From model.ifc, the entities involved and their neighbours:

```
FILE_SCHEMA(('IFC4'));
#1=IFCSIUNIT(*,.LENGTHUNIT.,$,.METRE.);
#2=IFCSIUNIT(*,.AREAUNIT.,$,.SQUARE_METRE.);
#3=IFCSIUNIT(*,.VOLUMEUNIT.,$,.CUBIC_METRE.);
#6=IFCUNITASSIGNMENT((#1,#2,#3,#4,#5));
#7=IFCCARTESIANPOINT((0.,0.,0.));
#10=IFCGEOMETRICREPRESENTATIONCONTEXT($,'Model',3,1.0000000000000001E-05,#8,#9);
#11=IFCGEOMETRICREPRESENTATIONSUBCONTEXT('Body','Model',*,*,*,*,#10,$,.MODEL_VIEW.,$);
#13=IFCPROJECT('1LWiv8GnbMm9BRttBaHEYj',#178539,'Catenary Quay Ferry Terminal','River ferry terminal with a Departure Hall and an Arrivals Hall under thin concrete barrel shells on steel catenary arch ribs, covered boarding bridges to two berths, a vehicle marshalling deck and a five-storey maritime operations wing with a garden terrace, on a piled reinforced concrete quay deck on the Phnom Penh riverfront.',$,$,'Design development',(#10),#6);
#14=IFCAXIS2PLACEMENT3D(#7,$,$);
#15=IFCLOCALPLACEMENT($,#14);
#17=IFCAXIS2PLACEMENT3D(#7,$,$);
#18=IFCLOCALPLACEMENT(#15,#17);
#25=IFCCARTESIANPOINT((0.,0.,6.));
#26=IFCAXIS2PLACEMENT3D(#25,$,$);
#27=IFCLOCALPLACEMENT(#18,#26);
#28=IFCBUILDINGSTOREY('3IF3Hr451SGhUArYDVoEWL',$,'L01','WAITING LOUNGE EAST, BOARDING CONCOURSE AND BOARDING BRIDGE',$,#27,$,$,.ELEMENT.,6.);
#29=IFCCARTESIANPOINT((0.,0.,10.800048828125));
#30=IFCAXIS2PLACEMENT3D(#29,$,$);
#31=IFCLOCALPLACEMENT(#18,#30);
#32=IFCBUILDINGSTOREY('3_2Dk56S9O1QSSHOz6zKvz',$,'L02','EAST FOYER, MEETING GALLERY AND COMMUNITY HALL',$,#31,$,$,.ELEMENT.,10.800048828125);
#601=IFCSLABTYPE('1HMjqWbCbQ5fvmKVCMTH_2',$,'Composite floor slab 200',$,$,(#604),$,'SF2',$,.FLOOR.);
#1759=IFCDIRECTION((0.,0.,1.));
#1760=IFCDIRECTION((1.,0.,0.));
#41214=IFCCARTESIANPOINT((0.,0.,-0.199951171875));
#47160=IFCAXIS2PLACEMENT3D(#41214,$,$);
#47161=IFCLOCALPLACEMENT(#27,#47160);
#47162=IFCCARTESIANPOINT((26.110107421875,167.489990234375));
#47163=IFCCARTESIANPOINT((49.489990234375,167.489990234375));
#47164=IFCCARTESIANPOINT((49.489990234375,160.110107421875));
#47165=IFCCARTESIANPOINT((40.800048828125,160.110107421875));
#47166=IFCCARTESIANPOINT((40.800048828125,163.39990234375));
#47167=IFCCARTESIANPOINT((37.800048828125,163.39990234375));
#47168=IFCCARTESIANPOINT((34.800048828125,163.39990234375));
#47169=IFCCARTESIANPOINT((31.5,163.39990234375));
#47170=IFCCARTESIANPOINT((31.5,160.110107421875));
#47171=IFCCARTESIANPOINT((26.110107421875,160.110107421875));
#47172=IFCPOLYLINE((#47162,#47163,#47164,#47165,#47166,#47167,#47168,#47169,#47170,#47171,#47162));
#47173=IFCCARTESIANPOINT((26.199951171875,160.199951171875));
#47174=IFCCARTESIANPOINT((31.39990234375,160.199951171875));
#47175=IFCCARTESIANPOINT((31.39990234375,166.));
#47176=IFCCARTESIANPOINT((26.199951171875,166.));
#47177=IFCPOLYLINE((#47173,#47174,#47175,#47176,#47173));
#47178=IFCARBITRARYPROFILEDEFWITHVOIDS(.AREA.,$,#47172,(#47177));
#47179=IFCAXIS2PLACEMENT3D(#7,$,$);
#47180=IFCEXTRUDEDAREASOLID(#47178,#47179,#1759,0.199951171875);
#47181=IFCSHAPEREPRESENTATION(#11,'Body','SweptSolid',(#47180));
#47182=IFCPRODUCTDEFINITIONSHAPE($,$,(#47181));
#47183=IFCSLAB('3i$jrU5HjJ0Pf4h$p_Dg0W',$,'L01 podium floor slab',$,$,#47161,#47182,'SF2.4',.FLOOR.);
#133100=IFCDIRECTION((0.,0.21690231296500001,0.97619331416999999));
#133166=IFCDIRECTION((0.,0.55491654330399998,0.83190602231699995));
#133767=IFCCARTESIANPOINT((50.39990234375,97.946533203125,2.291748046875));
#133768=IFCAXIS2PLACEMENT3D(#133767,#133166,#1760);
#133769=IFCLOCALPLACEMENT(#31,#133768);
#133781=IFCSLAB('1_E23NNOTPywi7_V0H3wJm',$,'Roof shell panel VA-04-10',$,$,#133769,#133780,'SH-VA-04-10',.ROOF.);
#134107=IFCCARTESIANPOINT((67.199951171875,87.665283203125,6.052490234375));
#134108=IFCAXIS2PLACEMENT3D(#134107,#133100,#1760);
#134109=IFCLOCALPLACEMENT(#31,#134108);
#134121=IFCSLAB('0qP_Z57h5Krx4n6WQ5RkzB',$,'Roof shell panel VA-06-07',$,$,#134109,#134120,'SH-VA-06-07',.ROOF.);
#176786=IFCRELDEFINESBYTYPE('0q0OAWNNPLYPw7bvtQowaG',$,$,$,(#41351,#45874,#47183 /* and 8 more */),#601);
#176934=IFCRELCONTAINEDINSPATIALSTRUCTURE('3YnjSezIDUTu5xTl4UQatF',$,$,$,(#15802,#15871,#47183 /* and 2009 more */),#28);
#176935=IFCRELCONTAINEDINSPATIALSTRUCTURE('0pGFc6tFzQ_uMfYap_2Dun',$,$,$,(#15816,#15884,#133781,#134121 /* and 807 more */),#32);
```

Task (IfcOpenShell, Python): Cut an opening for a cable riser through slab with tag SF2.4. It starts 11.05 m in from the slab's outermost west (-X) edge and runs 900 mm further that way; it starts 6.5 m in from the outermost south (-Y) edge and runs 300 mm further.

```python
import numpy as np
import ifcopenshell
import ifcopenshell.api.feature
import ifcopenshell.api.geometry
import ifcopenshell.api.root
import ifcopenshell.geom
import ifcopenshell.util.placement
import ifcopenshell.util.representation
import ifcopenshell.util.shape
import ifcopenshell.util.unit

model = ifcopenshell.open("model.ifc")
unit_scale = ifcopenshell.util.unit.calculate_unit_scale(model)
settings = ifcopenshell.geom.settings()


def volume(element):
    """Net volume in cubic metres, openings subtracted."""
    shape = ifcopenshell.geom.create_shape(settings, element)
    return ifcopenshell.util.shape.get_volume(shape.geometry)


slab = model.by_guid("3i$jrU5HjJ0Pf4h$p_Dg0W")
before = volume(slab)

# Extent in the slab's own axes, in metres. The edges named are its -X and -Y sides.
slab_shape = ifcopenshell.geom.create_shape(settings, slab)
vertices = ifcopenshell.util.shape.get_vertices(slab_shape.geometry)
x_min, y_min, bottom = vertices.min(axis=0)
top = vertices[:, 2].max()

opening = ifcopenshell.api.root.create_entity(model, ifc_class="IfcOpeningElement", name="Cable riser opening", predefined_type="OPENING")
context = ifcopenshell.util.representation.get_context(model, "Model", "Body", "MODEL_VIEW")
width, depth = 0.9, 0.3
outline = [(0.0, 0.0), (width, 0.0), (width, depth), (0.0, depth), (0.0, 0.0)]
# Overshoot both faces by 50 mm so the cut is clean.
shape = ifcopenshell.api.geometry.add_slab_representation(
    model, context=context, depth=top - bottom + 0.1, polyline=outline
)
ifcopenshell.api.geometry.assign_representation(model, product=opening, representation=shape)

matrix = ifcopenshell.util.placement.get_local_placement(slab.ObjectPlacement)
matrix[:, 3] = matrix @ np.append(np.array([x_min + 11.05, y_min + 6.5, bottom - 0.05]) / unit_scale, 1.0)
ifcopenshell.api.geometry.edit_object_placement(model, product=opening, matrix=matrix, is_si=False)
ifcopenshell.api.feature.add_feature(model, feature=opening, element=slab)

after = volume(slab)

print(f"slab volume {before:.3f} -> {after:.3f} m3")

model.write("model_v2.ifc")
```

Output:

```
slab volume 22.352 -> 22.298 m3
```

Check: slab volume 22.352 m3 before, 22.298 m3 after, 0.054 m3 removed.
